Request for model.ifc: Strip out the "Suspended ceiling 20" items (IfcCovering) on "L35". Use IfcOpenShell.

First a look at what the model holds.

```python
import ifcopenshell
import ifcopenshell.util.element

model = ifcopenshell.open("model.ifc")
print(model.schema)
storey = next(s for s in model.by_type("IfcBuildingStorey") if s.Name == "L35")
coverings = [e for e in ifcopenshell.util.element.get_decomposition(storey) if e.is_a("IfcCovering")]
seen = {}
for e in coverings:
    element_type = ifcopenshell.util.element.get_type(e)
    name = element_type.Name if element_type not in (None, e) else None
    seen[name] = seen.get(name, 0) + 1
for name, count in sorted(seen.items(), key=str):
    print(count, "x", name)
```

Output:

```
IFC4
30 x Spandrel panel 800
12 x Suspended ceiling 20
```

```python
import ifcopenshell
import ifcopenshell.api.root
import ifcopenshell.util.element

model = ifcopenshell.open("model.ifc")

storey = next(s for s in model.by_type("IfcBuildingStorey") if s.Name == "L35")
coverings = [e for e in ifcopenshell.util.element.get_decomposition(storey) if e.is_a("IfcCovering")]
targets = [e for e in coverings if (t := ifcopenshell.util.element.get_type(e)) not in (None, e) and t.Name == "Suspended ceiling 20"]

for e in targets:
    ifcopenshell.api.root.remove_product(model, product=e)
print(len(targets), "removed")

model.write("model-out.ifc")
```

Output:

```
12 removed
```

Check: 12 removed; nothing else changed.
